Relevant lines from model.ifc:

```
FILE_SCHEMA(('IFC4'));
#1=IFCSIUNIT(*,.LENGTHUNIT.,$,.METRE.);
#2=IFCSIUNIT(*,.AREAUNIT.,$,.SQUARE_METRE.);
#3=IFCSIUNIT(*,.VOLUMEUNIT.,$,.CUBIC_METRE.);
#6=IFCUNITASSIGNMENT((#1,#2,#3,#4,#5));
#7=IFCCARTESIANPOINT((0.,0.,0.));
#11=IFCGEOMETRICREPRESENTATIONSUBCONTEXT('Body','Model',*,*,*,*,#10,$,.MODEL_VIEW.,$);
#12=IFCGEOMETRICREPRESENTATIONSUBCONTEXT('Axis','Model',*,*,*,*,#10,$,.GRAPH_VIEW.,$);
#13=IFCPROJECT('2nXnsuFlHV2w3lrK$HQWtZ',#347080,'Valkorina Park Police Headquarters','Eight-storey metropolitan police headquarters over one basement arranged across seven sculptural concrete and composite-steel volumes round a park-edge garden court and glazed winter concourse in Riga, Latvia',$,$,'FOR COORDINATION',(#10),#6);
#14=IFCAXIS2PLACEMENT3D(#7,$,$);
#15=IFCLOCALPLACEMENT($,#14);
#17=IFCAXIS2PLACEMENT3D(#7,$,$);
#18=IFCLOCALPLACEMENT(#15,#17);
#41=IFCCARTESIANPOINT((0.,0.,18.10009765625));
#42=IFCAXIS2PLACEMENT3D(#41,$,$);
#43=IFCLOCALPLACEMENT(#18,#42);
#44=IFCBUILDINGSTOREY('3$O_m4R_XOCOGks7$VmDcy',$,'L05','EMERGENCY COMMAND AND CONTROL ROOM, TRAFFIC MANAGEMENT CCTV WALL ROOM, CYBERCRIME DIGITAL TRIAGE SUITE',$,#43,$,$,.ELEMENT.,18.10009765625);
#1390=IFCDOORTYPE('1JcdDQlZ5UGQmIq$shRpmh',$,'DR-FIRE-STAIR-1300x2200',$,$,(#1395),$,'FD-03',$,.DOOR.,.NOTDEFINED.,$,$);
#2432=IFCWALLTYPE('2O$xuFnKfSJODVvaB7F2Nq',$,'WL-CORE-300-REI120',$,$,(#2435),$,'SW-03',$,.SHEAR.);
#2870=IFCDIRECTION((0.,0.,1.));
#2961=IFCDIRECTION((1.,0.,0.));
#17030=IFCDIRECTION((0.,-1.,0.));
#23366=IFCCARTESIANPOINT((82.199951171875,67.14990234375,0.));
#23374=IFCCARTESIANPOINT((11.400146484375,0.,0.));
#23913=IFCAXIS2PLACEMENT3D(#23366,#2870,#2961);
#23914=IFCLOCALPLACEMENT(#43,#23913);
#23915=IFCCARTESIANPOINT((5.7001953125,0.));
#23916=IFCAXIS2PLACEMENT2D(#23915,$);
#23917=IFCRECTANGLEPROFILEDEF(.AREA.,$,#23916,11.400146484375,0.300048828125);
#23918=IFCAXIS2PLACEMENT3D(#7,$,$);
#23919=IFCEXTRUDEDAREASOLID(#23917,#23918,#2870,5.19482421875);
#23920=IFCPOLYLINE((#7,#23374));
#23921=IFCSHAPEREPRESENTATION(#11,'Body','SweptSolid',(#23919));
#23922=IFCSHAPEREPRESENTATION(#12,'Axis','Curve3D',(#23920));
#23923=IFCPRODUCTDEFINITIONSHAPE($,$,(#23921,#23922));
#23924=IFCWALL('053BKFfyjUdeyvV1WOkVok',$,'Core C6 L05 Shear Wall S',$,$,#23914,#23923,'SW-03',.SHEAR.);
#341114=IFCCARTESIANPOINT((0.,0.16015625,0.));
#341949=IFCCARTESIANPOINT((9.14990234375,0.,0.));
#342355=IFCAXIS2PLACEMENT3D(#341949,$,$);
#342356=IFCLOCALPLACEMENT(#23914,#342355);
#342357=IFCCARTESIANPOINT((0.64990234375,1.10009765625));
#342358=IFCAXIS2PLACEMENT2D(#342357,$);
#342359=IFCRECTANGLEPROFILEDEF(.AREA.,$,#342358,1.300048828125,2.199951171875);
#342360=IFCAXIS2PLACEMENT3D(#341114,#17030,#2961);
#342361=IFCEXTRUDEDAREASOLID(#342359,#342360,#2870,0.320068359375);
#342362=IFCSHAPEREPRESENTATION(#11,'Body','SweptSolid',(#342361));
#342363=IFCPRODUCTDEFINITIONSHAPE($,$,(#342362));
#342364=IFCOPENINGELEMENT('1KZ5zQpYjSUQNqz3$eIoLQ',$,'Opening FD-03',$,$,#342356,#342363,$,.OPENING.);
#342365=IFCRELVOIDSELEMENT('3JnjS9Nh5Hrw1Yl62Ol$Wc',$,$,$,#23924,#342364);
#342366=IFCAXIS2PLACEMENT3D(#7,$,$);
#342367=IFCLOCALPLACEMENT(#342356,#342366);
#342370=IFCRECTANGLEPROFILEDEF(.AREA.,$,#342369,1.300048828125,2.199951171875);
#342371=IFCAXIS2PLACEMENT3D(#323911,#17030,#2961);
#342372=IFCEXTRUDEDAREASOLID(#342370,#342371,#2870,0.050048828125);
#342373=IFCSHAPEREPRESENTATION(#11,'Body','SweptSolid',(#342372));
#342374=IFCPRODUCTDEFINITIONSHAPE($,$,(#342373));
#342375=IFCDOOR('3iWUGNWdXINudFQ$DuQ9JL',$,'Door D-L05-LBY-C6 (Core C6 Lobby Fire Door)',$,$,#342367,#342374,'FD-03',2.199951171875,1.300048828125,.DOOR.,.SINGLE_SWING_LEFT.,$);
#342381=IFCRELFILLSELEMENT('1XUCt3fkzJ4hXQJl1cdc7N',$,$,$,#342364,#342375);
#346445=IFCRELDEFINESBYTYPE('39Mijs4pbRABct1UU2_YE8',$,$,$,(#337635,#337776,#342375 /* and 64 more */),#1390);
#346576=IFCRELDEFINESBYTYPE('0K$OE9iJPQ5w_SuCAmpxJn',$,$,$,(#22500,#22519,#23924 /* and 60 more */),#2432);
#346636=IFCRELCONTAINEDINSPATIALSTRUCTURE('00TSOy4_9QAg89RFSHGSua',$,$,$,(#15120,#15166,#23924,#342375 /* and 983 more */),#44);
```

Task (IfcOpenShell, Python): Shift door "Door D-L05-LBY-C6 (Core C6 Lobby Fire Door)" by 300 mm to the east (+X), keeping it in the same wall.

```python
import ifcopenshell
import ifcopenshell.api.geometry
import ifcopenshell.util.placement

model = ifcopenshell.open("model.ifc")

door = model.by_guid("3iWUGNWdXINudFQ$DuQ9JL")
opening = door.FillsVoids[0].RelatingOpeningElement
wall = opening.VoidsElements[0].RelatingBuildingElement

wall_matrix = ifcopenshell.util.placement.get_local_placement(wall.ObjectPlacement)
shift = wall_matrix[:3, 0] * 0.3
before = ifcopenshell.util.placement.get_local_placement(door.ObjectPlacement)[:3, 3].copy()

# The door is placed relative to its opening, so it follows when the opening moves.
matrix = ifcopenshell.util.placement.get_local_placement(opening.ObjectPlacement)
matrix[:3, 3] += shift
ifcopenshell.api.geometry.edit_object_placement(
    model, product=opening, matrix=matrix, is_si=False, should_transform_children=True
)

after = ifcopenshell.util.placement.get_local_placement(door.ObjectPlacement)[:3, 3]
print("door moved by", (after - before).round(3) + 0.0)

model.write("model_rev.ifc")
```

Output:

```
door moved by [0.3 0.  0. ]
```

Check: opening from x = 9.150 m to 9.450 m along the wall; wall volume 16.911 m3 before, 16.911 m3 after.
